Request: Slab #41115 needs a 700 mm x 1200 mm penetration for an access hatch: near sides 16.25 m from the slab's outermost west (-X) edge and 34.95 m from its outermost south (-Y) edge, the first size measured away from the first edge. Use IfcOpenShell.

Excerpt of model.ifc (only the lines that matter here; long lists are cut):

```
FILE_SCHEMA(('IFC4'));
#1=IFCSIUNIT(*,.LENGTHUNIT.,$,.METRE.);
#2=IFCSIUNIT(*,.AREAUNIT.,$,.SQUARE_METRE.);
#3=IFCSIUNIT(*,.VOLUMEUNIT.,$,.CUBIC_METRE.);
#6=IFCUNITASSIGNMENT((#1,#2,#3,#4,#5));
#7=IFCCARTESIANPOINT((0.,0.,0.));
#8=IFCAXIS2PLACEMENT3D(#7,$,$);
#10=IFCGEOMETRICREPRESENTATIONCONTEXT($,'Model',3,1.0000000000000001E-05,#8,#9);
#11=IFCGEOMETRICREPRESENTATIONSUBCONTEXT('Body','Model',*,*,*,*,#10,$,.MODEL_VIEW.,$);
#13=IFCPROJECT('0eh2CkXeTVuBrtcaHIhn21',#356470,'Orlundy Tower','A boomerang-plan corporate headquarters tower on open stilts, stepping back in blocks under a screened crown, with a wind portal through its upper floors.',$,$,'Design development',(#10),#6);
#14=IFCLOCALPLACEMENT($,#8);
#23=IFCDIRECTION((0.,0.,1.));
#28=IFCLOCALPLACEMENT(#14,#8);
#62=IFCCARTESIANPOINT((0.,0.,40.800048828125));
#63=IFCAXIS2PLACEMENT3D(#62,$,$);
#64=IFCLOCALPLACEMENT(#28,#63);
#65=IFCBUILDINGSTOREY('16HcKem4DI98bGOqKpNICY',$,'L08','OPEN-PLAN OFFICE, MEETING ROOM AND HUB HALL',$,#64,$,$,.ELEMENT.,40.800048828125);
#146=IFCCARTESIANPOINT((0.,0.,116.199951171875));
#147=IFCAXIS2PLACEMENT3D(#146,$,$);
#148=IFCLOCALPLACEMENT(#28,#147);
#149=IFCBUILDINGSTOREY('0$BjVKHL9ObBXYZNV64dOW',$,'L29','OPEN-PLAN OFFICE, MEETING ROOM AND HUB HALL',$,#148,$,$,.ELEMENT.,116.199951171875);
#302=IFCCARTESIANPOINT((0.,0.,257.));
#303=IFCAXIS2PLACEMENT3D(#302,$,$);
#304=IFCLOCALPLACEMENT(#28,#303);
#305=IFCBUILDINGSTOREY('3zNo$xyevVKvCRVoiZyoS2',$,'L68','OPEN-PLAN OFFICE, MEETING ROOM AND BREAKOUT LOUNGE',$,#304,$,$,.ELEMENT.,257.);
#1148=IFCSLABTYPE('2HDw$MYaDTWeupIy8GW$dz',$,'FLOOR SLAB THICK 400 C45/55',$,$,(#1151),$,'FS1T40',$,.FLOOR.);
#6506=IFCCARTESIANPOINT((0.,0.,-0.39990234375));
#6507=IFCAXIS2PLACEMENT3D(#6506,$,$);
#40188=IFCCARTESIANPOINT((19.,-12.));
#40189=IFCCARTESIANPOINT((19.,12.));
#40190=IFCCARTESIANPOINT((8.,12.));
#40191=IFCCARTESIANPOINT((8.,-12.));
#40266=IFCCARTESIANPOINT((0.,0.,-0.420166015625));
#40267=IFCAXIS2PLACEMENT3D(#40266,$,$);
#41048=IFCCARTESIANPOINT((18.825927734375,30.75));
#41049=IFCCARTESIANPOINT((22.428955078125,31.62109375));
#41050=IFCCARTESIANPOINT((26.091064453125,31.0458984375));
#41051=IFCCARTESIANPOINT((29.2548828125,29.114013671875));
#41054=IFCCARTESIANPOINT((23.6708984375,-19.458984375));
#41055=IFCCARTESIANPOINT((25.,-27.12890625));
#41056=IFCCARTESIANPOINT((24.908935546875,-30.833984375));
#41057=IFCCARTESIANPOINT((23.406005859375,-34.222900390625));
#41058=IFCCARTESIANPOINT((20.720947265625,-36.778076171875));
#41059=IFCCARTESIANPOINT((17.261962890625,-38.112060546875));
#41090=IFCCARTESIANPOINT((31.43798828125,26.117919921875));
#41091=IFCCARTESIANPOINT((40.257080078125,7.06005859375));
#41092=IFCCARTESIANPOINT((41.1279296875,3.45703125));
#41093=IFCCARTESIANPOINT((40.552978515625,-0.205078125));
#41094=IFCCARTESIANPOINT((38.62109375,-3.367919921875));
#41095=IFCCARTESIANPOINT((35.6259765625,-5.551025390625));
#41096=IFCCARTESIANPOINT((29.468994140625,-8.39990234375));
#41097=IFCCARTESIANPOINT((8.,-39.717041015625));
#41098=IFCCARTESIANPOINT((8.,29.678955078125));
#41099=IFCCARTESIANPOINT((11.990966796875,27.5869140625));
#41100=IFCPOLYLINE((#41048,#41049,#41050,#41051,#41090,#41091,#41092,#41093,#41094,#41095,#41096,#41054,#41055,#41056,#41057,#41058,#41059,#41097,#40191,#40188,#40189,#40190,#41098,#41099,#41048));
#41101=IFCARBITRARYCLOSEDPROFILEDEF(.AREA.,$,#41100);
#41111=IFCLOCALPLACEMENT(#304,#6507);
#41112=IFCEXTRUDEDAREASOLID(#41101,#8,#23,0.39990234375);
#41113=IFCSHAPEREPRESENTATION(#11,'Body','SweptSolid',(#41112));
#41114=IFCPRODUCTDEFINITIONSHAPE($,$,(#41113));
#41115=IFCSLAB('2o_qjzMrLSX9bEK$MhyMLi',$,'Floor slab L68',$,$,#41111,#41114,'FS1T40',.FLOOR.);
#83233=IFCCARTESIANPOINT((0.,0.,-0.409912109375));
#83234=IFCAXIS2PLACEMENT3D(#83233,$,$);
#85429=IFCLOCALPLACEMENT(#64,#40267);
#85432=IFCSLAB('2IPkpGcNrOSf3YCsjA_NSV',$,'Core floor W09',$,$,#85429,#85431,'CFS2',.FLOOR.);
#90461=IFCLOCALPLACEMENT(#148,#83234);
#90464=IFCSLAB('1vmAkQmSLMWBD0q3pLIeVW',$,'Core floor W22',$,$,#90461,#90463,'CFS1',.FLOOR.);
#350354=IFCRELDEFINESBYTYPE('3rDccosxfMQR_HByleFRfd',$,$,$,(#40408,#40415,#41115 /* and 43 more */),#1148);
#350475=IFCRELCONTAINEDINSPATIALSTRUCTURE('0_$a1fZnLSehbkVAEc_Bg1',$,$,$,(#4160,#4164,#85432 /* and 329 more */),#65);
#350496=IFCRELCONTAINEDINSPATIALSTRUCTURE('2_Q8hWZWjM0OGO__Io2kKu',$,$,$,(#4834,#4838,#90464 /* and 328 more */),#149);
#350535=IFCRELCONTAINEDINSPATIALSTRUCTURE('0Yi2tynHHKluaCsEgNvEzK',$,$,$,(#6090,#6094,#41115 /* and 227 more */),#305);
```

```python
import numpy as np
import ifcopenshell
import ifcopenshell.api.feature
import ifcopenshell.api.geometry
import ifcopenshell.api.root
import ifcopenshell.geom
import ifcopenshell.util.placement
import ifcopenshell.util.representation
import ifcopenshell.util.shape
import ifcopenshell.util.unit

model = ifcopenshell.open("model.ifc")
unit_scale = ifcopenshell.util.unit.calculate_unit_scale(model)
settings = ifcopenshell.geom.settings()


def volume(element):
    """Net volume in cubic metres, openings subtracted."""
    shape = ifcopenshell.geom.create_shape(settings, element)
    return ifcopenshell.util.shape.get_volume(shape.geometry)


slab = model.by_id(41115)
before = volume(slab)

# Extent in the slab's own axes, in metres. The edges named are its -X and -Y sides.
slab_shape = ifcopenshell.geom.create_shape(settings, slab)
vertices = ifcopenshell.util.shape.get_vertices(slab_shape.geometry)
x_min, y_min, bottom = vertices.min(axis=0)
top = vertices[:, 2].max()

opening = ifcopenshell.api.root.create_entity(model, ifc_class="IfcOpeningElement", name="Access hatch opening", predefined_type="OPENING")
context = ifcopenshell.util.representation.get_context(model, "Model", "Body", "MODEL_VIEW")
width, depth = 0.7, 1.2
outline = [(0.0, 0.0), (width, 0.0), (width, depth), (0.0, depth), (0.0, 0.0)]
# Overshoot both faces by 50 mm so the cut is clean.
shape = ifcopenshell.api.geometry.add_slab_representation(
    model, context=context, depth=top - bottom + 0.1, polyline=outline
)
ifcopenshell.api.geometry.assign_representation(model, product=opening, representation=shape)

matrix = ifcopenshell.util.placement.get_local_placement(slab.ObjectPlacement)
matrix[:, 3] = matrix @ np.append(np.array([x_min + 16.25, y_min + 34.95, bottom - 0.05]) / unit_scale, 1.0)
ifcopenshell.api.geometry.edit_object_placement(model, product=opening, matrix=matrix, is_si=False)
ifcopenshell.api.feature.add_feature(model, feature=opening, element=slab)

after = volume(slab)

print(f"slab volume {before:.3f} -> {after:.3f} m3")

model.write("model_updated.ifc")
```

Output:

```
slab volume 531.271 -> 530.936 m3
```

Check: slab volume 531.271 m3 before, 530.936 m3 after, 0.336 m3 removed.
